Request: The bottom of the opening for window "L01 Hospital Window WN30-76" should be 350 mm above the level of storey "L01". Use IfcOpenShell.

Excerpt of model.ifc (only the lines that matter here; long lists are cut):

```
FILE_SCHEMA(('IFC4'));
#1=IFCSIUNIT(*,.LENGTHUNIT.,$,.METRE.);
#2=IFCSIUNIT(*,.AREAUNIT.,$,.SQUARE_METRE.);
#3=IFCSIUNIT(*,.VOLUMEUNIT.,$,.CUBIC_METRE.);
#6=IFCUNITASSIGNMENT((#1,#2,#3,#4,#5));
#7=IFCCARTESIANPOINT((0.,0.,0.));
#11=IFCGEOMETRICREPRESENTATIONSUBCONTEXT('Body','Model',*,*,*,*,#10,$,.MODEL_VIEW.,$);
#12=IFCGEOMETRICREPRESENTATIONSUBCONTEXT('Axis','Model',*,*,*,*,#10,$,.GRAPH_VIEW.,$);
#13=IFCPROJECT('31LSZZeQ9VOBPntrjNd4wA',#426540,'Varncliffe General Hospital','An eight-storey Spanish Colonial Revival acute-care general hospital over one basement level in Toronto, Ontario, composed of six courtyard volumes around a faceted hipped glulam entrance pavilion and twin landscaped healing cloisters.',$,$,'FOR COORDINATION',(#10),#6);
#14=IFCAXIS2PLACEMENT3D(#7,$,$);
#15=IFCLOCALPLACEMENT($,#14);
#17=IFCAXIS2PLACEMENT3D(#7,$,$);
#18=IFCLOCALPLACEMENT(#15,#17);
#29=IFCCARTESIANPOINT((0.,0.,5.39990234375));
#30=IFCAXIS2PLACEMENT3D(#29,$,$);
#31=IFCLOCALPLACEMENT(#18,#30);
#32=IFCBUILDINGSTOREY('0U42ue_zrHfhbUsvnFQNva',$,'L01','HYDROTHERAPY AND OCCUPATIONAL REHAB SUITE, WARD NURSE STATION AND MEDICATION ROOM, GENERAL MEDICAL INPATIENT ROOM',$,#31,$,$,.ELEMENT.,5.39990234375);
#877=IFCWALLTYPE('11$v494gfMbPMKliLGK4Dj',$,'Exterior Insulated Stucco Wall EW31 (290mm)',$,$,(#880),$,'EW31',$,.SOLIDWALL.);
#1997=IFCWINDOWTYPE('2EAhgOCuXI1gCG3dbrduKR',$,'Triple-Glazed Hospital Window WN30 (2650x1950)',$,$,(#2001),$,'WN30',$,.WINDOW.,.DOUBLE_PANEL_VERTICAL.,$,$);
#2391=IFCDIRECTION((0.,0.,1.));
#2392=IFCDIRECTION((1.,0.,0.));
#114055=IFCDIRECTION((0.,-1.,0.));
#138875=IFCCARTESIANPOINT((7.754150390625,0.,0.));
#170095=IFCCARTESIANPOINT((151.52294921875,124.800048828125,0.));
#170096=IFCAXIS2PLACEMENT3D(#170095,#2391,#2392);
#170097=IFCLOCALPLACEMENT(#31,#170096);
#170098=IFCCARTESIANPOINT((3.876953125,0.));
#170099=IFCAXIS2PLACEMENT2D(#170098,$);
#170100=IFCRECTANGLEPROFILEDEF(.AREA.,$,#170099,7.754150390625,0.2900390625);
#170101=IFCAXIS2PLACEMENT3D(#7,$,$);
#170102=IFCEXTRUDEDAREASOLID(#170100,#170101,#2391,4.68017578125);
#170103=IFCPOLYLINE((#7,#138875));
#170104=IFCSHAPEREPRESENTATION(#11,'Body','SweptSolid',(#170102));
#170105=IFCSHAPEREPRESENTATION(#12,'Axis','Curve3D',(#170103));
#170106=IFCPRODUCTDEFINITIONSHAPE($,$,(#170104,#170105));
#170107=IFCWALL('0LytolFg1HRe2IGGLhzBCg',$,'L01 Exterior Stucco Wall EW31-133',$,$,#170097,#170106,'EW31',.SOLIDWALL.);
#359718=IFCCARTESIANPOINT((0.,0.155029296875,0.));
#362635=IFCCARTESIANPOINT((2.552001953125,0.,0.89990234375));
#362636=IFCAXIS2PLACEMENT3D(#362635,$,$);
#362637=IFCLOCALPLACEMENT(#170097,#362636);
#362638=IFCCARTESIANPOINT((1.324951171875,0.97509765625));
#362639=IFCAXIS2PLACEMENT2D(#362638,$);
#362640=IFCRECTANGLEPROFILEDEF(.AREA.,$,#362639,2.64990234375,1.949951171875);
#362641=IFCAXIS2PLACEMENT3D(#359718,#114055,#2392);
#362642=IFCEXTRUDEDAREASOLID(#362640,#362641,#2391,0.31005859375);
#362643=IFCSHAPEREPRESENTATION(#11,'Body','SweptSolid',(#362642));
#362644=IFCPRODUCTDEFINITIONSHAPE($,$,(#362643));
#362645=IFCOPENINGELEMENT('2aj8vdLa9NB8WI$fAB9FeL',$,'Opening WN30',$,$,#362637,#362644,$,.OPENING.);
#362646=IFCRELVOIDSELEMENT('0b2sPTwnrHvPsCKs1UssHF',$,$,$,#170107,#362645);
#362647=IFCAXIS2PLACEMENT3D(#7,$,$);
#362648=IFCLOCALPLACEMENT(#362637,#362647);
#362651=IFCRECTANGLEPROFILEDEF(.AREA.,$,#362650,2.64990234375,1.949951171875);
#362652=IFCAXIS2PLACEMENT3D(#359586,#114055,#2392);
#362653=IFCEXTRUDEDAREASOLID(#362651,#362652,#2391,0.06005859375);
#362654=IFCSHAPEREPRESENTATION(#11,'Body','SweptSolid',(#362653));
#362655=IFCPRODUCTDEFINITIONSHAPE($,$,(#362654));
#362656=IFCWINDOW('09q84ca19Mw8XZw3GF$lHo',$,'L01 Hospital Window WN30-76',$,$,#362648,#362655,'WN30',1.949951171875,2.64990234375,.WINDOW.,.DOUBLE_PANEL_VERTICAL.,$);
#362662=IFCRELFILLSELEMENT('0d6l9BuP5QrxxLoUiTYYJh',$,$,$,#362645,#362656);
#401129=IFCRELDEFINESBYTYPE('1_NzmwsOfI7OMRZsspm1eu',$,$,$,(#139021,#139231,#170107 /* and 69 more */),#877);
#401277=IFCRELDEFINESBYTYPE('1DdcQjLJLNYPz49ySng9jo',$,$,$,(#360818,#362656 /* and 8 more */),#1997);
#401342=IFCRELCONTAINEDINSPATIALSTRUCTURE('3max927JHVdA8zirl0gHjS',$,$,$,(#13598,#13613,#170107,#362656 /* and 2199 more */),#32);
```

```python
import numpy as np
import ifcopenshell
import ifcopenshell.api.geometry
import ifcopenshell.geom
import ifcopenshell.util.element
import ifcopenshell.util.placement
import ifcopenshell.util.shape
import ifcopenshell.util.unit

model = ifcopenshell.open("model.ifc")
unit_scale = ifcopenshell.util.unit.calculate_unit_scale(model)

window = model.by_guid("09q84ca19Mw8XZw3GF$lHo")
opening = window.FillsVoids[0].RelatingOpeningElement
storey = ifcopenshell.util.element.get_container(window, ifc_class="IfcBuildingStorey")
level = ifcopenshell.util.placement.get_local_placement(storey.ObjectPlacement)[2, 3]

# The opening's origin need not be at the sill, so measure its lowest point.
shape = ifcopenshell.geom.create_shape(ifcopenshell.geom.settings(), opening)
bottom = ifcopenshell.util.shape.get_shape_bottom_elevation(shape, shape.geometry) / unit_scale
dz = level + 0.35 / unit_scale - bottom

shift = np.array([0.0, 0.0, dz])
# The window is placed relative to its opening, so it follows when the opening moves.
matrix = ifcopenshell.util.placement.get_local_placement(opening.ObjectPlacement)
matrix[:3, 3] += shift
ifcopenshell.api.geometry.edit_object_placement(
    model, product=opening, matrix=matrix, is_si=False, should_transform_children=True
)

print(f"moved by {dz * unit_scale:+.3f} m")

model.write("model_edited.ifc")
```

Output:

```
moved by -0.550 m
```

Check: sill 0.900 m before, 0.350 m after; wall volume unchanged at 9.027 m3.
